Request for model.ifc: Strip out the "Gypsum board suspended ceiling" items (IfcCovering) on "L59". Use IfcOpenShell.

First a look at what the model holds.

```python
import ifcopenshell
import ifcopenshell.util.element

model = ifcopenshell.open("model.ifc")
print(model.schema)
storey = next(s for s in model.by_type("IfcBuildingStorey") if s.Name == "L59")
coverings = [e for e in ifcopenshell.util.element.get_decomposition(storey) if e.is_a("IfcCovering")]
seen = {}
for e in coverings:
    element_type = ifcopenshell.util.element.get_type(e)
    name = element_type.Name if element_type not in (None, e) else None
    seen[name] = seen.get(name, 0) + 1
for name, count in sorted(seen.items(), key=str):
    print(count, "x", name)
```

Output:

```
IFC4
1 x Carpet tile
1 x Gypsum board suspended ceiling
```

```python
import ifcopenshell
import ifcopenshell.api.root
import ifcopenshell.util.element

model = ifcopenshell.open("model.ifc")

storey = next(s for s in model.by_type("IfcBuildingStorey") if s.Name == "L59")
coverings = [e for e in ifcopenshell.util.element.get_decomposition(storey) if e.is_a("IfcCovering")]
targets = [e for e in coverings if (t := ifcopenshell.util.element.get_type(e)) not in (None, e) and t.Name == "Gypsum board suspended ceiling"]

for e in targets:
    ifcopenshell.api.root.remove_product(model, product=e)
print(len(targets), "removed")

model.write("model_rev.ifc")
```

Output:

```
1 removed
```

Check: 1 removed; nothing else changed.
